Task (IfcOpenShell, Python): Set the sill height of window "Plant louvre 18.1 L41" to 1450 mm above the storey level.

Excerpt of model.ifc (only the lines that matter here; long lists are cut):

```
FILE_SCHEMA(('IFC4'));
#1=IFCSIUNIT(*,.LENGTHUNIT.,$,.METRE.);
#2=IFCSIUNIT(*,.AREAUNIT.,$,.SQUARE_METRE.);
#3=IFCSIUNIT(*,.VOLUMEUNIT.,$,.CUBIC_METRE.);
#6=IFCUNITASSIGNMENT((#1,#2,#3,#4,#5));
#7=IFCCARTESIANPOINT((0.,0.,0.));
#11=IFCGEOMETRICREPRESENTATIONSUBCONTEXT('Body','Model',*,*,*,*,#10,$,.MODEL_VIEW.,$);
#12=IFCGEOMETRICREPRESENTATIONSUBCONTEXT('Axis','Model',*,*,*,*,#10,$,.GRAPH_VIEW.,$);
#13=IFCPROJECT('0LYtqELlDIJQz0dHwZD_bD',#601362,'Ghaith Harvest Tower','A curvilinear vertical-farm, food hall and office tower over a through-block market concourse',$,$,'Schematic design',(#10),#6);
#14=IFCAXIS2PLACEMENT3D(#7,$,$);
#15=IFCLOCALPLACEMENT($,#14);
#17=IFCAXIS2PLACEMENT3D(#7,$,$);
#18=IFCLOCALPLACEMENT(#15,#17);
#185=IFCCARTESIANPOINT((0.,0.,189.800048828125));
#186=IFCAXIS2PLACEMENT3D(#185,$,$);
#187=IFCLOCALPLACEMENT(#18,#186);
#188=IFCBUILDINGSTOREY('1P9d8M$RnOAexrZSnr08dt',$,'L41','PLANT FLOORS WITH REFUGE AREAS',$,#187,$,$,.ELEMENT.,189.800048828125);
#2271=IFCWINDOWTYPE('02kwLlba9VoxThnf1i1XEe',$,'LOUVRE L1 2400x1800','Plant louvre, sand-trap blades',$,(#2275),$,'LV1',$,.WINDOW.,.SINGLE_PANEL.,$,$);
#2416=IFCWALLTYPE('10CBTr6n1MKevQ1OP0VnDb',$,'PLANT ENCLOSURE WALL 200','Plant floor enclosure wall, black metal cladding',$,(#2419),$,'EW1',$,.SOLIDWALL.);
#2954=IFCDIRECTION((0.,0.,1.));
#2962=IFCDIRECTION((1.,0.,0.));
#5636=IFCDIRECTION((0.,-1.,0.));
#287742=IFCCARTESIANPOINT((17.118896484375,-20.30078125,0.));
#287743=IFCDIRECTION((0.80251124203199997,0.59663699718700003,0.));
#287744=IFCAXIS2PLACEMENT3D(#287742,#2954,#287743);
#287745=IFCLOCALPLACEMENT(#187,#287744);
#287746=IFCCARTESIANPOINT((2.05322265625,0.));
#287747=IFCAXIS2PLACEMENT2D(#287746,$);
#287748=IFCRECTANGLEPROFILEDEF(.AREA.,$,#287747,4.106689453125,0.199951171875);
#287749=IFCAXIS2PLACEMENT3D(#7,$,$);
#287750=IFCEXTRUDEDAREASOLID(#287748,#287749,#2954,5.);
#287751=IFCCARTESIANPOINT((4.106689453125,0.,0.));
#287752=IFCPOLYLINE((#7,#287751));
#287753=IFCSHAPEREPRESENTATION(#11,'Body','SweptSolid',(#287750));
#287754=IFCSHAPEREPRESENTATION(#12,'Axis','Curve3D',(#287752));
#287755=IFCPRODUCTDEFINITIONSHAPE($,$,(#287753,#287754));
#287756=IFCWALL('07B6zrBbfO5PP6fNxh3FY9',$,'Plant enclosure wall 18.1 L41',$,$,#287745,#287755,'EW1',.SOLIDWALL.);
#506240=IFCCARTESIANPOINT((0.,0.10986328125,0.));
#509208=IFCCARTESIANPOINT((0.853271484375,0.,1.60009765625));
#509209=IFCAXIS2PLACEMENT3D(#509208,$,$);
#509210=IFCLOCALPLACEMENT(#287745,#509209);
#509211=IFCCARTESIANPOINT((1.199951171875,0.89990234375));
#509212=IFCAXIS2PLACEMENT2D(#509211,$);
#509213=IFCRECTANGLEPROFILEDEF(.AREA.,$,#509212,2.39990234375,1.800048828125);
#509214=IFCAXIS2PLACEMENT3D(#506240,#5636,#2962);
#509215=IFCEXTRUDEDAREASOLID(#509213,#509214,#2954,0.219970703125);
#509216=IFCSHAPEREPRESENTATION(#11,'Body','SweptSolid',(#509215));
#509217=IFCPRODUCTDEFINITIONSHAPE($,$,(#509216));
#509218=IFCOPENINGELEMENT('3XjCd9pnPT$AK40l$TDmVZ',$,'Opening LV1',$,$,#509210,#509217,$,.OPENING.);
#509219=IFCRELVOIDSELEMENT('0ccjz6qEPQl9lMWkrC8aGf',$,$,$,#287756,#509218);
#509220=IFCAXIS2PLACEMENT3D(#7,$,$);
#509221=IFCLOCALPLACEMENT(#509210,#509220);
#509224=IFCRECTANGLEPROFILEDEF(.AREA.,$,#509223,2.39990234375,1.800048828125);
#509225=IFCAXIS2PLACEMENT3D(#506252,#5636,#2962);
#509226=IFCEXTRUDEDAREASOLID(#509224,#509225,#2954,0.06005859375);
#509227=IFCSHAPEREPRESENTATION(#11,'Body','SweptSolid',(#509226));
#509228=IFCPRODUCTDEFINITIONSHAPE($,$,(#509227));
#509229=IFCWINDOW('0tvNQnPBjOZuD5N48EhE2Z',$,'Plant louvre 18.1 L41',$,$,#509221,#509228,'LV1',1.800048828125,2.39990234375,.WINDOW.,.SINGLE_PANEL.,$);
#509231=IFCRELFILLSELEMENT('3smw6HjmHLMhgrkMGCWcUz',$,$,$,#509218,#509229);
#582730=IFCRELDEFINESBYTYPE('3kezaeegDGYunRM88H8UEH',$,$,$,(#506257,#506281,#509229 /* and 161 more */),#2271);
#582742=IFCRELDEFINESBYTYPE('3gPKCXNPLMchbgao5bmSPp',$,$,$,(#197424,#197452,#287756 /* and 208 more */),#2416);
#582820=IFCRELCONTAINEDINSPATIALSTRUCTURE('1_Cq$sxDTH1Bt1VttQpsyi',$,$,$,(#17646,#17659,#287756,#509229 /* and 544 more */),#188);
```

```python
import numpy as np
import ifcopenshell
import ifcopenshell.api.geometry
import ifcopenshell.geom
import ifcopenshell.util.element
import ifcopenshell.util.placement
import ifcopenshell.util.shape
import ifcopenshell.util.unit

model = ifcopenshell.open("model.ifc")
unit_scale = ifcopenshell.util.unit.calculate_unit_scale(model)

window = model.by_guid("0tvNQnPBjOZuD5N48EhE2Z")
opening = window.FillsVoids[0].RelatingOpeningElement
storey = ifcopenshell.util.element.get_container(window, ifc_class="IfcBuildingStorey")
level = ifcopenshell.util.placement.get_local_placement(storey.ObjectPlacement)[2, 3]

# The opening's origin need not be at the sill, so measure its lowest point.
shape = ifcopenshell.geom.create_shape(ifcopenshell.geom.settings(), opening)
bottom = ifcopenshell.util.shape.get_shape_bottom_elevation(shape, shape.geometry) / unit_scale
dz = level + 1.45 - bottom

shift = np.array([0.0, 0.0, dz])
# The window is placed relative to its opening, so it follows when the opening moves.
matrix = ifcopenshell.util.placement.get_local_placement(opening.ObjectPlacement)
matrix[:3, 3] += shift
ifcopenshell.api.geometry.edit_object_placement(
    model, product=opening, matrix=matrix, is_si=False, should_transform_children=True
)

print(f"moved by {dz * unit_scale:+.3f} m")

model.write("model_rev.ifc")
```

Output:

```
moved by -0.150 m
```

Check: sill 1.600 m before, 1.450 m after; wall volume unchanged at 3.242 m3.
